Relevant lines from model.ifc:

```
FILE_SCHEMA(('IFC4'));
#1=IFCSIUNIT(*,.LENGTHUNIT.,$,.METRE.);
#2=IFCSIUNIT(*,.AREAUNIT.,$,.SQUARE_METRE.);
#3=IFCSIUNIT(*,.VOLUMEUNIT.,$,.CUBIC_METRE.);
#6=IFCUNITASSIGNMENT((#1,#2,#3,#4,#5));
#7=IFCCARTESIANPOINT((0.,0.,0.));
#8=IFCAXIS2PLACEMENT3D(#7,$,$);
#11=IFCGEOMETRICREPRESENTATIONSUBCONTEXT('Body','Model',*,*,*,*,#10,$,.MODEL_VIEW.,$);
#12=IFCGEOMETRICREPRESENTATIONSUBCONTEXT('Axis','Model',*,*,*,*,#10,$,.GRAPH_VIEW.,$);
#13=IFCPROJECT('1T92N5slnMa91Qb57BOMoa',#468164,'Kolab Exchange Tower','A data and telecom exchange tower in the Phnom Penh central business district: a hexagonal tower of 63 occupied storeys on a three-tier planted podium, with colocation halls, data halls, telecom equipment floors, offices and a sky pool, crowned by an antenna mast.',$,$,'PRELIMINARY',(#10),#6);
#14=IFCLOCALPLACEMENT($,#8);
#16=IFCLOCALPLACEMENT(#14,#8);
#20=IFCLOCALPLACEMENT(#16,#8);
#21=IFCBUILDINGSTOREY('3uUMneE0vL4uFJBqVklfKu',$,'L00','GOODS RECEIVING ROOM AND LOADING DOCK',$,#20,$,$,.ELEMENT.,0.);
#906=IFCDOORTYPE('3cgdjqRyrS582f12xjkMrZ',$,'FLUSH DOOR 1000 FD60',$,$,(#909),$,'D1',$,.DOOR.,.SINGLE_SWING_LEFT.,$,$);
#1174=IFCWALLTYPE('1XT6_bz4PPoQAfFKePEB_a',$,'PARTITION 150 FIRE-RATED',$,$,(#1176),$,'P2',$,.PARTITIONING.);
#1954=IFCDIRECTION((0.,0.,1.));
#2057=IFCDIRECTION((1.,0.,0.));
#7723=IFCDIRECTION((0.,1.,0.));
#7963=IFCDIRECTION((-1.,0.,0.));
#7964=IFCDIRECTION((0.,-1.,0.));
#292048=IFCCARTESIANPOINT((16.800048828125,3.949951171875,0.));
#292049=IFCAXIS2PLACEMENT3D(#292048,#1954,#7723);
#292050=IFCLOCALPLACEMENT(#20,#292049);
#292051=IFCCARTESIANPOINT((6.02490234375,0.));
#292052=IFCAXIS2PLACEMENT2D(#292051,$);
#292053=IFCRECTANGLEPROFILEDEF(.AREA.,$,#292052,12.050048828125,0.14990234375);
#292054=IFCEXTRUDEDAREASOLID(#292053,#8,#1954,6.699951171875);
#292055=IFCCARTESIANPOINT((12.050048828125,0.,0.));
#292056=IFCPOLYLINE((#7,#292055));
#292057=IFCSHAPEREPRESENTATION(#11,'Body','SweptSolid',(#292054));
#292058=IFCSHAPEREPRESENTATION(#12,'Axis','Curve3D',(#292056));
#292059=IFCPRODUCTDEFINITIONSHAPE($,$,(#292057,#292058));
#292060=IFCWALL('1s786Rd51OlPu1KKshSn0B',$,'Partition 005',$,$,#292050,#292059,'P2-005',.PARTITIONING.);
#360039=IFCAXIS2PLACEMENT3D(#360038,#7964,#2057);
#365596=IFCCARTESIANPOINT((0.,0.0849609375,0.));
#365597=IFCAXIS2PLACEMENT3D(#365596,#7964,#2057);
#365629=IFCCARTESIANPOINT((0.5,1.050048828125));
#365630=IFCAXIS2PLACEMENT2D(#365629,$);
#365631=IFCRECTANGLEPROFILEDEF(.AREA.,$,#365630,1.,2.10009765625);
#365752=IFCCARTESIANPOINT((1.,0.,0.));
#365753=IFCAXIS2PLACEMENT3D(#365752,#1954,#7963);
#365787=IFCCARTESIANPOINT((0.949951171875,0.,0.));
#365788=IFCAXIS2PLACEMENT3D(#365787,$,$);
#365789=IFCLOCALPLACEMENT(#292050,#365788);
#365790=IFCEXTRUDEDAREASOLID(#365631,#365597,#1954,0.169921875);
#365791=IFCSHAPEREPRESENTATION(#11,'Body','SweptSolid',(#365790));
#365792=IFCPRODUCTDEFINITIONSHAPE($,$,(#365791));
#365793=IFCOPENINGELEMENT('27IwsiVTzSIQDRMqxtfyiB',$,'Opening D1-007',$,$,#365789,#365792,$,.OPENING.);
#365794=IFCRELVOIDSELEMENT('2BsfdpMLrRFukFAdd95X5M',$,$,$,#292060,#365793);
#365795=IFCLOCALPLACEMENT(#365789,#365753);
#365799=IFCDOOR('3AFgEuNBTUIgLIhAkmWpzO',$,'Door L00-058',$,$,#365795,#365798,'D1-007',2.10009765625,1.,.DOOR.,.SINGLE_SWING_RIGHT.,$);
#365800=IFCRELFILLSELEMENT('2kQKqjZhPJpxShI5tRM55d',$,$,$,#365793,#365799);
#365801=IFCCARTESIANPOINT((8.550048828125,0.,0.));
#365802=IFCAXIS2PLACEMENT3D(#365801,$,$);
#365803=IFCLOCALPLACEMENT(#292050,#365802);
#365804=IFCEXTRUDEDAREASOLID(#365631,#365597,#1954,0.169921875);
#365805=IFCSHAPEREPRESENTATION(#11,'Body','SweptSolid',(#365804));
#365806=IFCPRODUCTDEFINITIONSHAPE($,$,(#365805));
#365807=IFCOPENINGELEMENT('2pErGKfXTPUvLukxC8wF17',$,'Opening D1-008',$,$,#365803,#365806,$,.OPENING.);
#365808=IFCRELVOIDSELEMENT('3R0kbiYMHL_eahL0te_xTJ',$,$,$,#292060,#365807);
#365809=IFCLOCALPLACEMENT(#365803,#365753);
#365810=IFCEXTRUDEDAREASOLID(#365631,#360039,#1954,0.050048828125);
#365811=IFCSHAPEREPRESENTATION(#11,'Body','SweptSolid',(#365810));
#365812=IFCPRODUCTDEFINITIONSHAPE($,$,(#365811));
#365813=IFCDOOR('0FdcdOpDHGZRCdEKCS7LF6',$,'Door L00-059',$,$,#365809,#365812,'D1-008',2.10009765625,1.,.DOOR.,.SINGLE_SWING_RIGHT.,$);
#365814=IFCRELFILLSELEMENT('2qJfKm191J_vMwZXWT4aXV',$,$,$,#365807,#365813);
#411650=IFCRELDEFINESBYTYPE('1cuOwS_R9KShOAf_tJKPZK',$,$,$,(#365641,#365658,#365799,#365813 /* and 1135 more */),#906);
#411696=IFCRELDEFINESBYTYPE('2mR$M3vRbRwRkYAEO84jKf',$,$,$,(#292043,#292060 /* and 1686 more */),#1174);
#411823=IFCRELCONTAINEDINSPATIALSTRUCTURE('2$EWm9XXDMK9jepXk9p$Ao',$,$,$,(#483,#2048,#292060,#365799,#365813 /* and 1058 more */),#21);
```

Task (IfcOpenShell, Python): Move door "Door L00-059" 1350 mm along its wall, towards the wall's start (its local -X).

```python
import ifcopenshell
import ifcopenshell.api.geometry
import ifcopenshell.util.placement

model = ifcopenshell.open("model.ifc")

door = model.by_guid("0FdcdOpDHGZRCdEKCS7LF6")
opening = door.FillsVoids[0].RelatingOpeningElement
wall = opening.VoidsElements[0].RelatingBuildingElement

wall_matrix = ifcopenshell.util.placement.get_local_placement(wall.ObjectPlacement)
shift = wall_matrix[:3, 0] * -1.35
before = ifcopenshell.util.placement.get_local_placement(door.ObjectPlacement)[:3, 3].copy()

# The door is placed relative to its opening, so it follows when the opening moves.
matrix = ifcopenshell.util.placement.get_local_placement(opening.ObjectPlacement)
matrix[:3, 3] += shift
ifcopenshell.api.geometry.edit_object_placement(
    model, product=opening, matrix=matrix, is_si=False, should_transform_children=True
)

after = ifcopenshell.util.placement.get_local_placement(door.ObjectPlacement)[:3, 3]
print("door moved by", (after - before).round(3) + 0.0)

model.write("model-out.ifc")
```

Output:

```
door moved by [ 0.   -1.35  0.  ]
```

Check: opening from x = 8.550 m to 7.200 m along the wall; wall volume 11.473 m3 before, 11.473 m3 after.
